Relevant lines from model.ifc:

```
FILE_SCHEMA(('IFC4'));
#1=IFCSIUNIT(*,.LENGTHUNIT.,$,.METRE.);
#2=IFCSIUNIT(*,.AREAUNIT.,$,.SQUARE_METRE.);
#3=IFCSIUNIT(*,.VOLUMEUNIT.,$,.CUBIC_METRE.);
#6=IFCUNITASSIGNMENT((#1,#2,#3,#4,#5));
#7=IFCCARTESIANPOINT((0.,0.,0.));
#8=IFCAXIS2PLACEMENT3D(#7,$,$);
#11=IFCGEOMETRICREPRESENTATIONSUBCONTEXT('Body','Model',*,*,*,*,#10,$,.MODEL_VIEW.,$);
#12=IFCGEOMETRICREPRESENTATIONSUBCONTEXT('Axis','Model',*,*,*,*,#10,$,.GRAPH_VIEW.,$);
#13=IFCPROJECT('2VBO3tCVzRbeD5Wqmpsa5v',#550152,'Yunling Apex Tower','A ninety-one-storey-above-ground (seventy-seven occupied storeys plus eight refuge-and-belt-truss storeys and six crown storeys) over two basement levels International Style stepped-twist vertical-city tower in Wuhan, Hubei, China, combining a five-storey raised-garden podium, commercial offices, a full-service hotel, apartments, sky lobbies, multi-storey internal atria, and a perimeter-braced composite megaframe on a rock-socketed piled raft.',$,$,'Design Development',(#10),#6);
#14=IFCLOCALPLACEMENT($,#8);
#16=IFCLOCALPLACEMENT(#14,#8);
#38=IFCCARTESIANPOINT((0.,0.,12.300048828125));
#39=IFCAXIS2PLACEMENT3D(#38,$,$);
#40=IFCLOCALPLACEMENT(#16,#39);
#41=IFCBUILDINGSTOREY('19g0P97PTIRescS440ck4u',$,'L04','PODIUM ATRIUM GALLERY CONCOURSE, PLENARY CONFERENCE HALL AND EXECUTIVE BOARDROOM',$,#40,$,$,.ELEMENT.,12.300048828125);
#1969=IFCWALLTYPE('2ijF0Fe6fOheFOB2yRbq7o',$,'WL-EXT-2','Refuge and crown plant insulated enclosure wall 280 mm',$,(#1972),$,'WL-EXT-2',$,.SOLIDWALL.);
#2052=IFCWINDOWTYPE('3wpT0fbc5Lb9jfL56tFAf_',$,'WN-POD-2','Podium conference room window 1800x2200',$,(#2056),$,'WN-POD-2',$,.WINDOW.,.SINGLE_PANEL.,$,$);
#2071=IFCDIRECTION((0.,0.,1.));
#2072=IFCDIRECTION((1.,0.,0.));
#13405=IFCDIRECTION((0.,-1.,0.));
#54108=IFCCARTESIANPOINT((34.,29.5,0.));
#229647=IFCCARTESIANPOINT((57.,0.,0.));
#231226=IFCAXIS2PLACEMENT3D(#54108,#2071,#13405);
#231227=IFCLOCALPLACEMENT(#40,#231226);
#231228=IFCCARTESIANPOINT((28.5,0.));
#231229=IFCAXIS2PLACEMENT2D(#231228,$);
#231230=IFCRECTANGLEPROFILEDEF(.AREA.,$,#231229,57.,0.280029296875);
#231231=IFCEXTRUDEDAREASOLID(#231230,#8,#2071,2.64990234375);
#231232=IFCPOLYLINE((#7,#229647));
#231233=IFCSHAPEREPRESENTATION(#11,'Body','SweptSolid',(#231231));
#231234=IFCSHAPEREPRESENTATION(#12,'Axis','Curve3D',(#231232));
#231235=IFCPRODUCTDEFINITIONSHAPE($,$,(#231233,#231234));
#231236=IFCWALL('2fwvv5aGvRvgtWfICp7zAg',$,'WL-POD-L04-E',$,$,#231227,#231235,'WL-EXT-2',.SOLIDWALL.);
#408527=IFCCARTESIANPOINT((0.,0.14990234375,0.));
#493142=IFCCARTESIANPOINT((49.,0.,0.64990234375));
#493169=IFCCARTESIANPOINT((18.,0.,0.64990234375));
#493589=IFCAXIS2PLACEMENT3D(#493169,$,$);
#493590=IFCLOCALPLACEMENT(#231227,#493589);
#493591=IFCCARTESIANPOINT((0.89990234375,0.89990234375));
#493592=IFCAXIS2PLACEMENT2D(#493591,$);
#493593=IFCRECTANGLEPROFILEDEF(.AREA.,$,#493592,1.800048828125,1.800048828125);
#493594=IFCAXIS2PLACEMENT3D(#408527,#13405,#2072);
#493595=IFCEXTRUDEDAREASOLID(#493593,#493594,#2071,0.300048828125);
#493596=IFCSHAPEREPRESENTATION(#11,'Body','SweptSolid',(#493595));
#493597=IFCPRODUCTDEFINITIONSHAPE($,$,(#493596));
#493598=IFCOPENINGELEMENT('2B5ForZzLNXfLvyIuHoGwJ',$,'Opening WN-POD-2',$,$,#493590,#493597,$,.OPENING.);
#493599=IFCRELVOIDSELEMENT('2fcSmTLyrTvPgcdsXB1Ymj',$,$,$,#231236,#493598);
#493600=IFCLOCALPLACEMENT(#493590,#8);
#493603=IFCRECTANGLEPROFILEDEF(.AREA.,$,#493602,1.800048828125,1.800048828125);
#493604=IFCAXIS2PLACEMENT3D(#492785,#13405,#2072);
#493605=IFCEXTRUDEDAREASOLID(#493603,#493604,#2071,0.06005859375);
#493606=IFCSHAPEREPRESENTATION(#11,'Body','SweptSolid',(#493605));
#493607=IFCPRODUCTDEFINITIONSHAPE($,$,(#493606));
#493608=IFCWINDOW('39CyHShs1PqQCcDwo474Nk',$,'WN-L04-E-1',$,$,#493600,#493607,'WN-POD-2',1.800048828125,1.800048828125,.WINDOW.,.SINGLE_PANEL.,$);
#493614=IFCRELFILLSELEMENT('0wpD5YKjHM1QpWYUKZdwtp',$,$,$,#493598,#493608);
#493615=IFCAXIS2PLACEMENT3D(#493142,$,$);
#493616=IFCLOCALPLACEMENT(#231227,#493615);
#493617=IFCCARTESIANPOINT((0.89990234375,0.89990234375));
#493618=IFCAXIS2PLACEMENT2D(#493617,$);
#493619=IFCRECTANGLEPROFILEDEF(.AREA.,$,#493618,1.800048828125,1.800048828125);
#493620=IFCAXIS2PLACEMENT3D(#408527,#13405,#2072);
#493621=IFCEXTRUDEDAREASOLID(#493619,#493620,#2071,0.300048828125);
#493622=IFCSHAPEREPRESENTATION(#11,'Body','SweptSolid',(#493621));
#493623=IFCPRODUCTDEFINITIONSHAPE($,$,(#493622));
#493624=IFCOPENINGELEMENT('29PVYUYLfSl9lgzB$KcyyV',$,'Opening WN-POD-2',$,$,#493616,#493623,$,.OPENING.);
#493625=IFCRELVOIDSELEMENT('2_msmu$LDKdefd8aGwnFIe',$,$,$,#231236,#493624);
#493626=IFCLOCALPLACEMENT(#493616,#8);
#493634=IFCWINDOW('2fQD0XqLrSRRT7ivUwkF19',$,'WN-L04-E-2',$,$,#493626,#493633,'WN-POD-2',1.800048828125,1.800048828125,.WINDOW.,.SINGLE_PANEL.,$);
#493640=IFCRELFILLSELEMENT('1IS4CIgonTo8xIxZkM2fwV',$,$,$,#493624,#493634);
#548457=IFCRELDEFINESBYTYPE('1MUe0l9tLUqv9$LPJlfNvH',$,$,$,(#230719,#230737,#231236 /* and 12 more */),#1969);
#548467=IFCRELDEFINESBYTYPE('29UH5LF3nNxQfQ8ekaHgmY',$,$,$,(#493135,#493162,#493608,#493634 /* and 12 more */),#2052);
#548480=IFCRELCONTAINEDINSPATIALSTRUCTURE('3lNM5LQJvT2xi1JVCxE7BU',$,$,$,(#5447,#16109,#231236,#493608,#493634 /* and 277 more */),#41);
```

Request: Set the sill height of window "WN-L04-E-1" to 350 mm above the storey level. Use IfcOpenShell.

```python
import numpy as np
import ifcopenshell
import ifcopenshell.api.geometry
import ifcopenshell.geom
import ifcopenshell.util.element
import ifcopenshell.util.placement
import ifcopenshell.util.shape
import ifcopenshell.util.unit

model = ifcopenshell.open("model.ifc")
unit_scale = ifcopenshell.util.unit.calculate_unit_scale(model)

window = model.by_guid("39CyHShs1PqQCcDwo474Nk")
opening = window.FillsVoids[0].RelatingOpeningElement
storey = ifcopenshell.util.element.get_container(window, ifc_class="IfcBuildingStorey")
level = ifcopenshell.util.placement.get_local_placement(storey.ObjectPlacement)[2, 3]

# The opening's origin need not be at the sill, so measure its lowest point.
shape = ifcopenshell.geom.create_shape(ifcopenshell.geom.settings(), opening)
bottom = ifcopenshell.util.shape.get_shape_bottom_elevation(shape, shape.geometry) / unit_scale
dz = level + 0.35 - bottom

shift = np.array([0.0, 0.0, dz])
# The window is placed relative to its opening, so it follows when the opening moves.
matrix = ifcopenshell.util.placement.get_local_placement(opening.ObjectPlacement)
matrix[:3, 3] += shift
ifcopenshell.api.geometry.edit_object_placement(
    model, product=opening, matrix=matrix, is_si=False, should_transform_children=True
)

print(f"moved by {dz * unit_scale:+.3f} m")

model.write("model_v2.ifc")
```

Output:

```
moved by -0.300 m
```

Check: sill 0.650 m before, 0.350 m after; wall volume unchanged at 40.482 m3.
